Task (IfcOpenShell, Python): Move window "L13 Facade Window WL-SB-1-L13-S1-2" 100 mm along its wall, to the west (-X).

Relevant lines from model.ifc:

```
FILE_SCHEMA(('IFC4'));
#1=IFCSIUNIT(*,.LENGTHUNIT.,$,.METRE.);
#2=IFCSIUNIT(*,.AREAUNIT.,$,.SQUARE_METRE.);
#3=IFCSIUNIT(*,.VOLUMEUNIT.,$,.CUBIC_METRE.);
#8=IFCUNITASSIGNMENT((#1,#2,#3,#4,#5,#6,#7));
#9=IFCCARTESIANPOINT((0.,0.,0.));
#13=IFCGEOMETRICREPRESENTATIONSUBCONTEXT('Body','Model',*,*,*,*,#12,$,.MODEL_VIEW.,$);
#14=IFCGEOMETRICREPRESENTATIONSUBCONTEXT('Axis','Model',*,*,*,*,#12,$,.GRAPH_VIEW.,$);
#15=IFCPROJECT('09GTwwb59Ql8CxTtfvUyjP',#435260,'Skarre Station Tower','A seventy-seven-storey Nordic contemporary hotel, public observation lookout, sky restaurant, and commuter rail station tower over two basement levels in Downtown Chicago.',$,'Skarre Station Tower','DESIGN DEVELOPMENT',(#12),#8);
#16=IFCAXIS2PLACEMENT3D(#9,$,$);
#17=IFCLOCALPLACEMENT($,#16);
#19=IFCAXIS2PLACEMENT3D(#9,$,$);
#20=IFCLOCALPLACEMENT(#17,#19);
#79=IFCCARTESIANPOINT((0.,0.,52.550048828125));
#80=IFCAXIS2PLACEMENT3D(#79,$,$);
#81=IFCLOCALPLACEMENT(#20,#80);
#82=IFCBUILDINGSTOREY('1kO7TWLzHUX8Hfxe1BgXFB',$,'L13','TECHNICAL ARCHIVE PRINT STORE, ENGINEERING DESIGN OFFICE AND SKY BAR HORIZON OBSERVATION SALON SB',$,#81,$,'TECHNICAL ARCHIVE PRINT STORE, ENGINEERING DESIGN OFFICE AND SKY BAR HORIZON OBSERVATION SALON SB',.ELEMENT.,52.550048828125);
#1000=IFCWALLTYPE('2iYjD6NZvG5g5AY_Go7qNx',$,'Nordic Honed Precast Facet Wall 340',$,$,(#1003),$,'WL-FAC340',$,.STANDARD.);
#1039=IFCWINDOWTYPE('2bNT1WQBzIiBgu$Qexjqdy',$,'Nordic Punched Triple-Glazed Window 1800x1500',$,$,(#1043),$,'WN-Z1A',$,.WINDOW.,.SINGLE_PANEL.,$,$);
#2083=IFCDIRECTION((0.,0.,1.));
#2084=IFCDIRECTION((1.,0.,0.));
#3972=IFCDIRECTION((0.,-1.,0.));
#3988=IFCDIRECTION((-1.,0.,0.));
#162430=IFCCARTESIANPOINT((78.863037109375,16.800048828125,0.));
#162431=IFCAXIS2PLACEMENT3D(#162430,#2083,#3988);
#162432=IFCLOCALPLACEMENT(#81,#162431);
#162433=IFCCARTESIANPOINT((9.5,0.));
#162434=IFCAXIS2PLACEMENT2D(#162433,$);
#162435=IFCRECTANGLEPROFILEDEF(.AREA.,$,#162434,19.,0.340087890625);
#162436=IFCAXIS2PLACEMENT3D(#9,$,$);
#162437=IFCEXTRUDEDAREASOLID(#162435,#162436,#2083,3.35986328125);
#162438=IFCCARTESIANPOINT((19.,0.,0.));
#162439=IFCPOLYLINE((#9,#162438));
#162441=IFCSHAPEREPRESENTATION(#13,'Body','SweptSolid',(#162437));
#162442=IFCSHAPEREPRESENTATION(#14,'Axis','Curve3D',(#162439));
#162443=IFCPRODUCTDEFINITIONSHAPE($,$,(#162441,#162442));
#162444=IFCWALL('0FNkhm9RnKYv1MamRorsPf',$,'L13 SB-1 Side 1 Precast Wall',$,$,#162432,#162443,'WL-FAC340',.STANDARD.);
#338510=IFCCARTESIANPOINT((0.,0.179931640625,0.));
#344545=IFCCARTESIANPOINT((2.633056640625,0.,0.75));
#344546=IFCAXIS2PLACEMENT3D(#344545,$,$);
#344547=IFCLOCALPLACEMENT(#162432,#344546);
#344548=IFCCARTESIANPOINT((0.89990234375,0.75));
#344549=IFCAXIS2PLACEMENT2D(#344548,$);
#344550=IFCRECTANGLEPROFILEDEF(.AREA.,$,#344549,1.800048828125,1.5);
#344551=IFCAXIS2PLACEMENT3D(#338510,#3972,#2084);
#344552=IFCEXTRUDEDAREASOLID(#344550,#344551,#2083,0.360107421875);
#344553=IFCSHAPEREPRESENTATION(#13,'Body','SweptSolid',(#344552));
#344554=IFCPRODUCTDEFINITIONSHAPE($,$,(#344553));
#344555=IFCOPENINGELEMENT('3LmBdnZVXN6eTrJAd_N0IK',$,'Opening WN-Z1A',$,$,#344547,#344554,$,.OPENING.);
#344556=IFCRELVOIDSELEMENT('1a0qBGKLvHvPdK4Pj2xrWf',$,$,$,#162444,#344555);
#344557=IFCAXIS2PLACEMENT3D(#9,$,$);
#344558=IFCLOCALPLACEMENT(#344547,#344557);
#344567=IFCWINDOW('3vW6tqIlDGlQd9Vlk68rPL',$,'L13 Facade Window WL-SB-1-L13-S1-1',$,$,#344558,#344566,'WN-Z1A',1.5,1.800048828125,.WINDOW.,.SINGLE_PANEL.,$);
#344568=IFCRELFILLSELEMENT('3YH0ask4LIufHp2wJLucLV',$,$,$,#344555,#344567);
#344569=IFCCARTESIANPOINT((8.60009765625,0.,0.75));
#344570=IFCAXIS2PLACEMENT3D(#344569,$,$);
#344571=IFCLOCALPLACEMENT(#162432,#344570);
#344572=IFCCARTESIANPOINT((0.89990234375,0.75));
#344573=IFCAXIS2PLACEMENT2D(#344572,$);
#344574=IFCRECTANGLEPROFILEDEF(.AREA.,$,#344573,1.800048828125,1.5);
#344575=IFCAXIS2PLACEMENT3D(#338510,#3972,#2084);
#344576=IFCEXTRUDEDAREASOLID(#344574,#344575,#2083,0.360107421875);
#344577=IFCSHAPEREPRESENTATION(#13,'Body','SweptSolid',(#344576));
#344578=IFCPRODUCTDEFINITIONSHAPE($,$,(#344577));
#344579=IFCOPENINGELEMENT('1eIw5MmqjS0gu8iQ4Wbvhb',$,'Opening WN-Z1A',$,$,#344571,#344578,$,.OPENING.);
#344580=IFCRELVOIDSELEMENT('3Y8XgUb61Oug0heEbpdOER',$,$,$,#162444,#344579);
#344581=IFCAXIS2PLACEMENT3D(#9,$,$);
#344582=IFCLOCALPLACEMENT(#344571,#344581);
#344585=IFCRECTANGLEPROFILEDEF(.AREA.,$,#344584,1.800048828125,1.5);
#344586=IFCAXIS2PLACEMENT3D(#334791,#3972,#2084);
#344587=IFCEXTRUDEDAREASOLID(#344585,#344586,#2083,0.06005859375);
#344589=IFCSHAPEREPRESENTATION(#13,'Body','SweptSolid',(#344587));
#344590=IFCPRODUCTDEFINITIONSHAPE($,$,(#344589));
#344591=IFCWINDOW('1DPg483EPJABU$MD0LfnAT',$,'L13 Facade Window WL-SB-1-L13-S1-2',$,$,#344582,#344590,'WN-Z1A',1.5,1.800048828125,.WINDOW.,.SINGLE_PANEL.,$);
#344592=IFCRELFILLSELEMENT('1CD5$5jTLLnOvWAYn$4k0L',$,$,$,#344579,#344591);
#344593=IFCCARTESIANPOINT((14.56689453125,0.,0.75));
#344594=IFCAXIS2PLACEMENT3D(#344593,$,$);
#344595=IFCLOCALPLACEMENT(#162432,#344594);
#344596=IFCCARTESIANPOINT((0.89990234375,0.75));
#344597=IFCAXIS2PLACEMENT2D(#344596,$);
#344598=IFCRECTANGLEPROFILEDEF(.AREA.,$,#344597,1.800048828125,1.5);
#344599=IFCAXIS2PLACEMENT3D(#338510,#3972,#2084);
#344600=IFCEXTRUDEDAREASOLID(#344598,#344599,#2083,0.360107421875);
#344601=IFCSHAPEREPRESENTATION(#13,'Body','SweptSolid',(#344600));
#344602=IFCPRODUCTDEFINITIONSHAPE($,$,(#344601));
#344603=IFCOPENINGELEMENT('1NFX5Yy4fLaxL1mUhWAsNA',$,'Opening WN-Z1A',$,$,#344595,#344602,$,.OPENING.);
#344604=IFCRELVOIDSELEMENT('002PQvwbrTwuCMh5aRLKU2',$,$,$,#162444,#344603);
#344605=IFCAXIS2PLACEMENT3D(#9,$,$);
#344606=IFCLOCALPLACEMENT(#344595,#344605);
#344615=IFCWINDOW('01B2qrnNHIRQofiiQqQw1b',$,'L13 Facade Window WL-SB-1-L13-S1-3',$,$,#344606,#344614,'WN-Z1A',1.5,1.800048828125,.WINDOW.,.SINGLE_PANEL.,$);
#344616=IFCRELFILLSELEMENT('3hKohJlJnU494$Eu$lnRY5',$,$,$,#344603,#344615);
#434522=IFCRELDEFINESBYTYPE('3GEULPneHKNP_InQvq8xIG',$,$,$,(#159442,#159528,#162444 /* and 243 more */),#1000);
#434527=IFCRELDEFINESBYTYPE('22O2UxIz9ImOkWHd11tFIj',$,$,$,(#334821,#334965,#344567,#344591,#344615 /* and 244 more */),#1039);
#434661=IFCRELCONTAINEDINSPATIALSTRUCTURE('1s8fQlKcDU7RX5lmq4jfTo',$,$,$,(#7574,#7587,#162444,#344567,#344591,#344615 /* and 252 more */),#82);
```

```python
import ifcopenshell
import ifcopenshell.api.geometry
import ifcopenshell.util.placement
import ifcopenshell.util.unit

model = ifcopenshell.open("model.ifc")
unit_scale = ifcopenshell.util.unit.calculate_unit_scale(model)

window = model.by_guid("1DPg483EPJABU$MD0LfnAT")
opening = window.FillsVoids[0].RelatingOpeningElement
wall = opening.VoidsElements[0].RelatingBuildingElement

wall_matrix = ifcopenshell.util.placement.get_local_placement(wall.ObjectPlacement)
shift = wall_matrix[:3, 0] * 0.1 / unit_scale
before = ifcopenshell.util.placement.get_local_placement(window.ObjectPlacement)[:3, 3].copy()

# The window is placed relative to its opening, so it follows when the opening moves.
matrix = ifcopenshell.util.placement.get_local_placement(opening.ObjectPlacement)
matrix[:3, 3] += shift
ifcopenshell.api.geometry.edit_object_placement(
    model, product=opening, matrix=matrix, is_si=False, should_transform_children=True
)

after = ifcopenshell.util.placement.get_local_placement(window.ObjectPlacement)[:3, 3]
print("window moved by", (after - before).round(3) + 0.0)

model.write("model_edited.ifc")
```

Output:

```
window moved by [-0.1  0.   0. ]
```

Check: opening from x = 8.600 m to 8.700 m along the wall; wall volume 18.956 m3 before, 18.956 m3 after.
